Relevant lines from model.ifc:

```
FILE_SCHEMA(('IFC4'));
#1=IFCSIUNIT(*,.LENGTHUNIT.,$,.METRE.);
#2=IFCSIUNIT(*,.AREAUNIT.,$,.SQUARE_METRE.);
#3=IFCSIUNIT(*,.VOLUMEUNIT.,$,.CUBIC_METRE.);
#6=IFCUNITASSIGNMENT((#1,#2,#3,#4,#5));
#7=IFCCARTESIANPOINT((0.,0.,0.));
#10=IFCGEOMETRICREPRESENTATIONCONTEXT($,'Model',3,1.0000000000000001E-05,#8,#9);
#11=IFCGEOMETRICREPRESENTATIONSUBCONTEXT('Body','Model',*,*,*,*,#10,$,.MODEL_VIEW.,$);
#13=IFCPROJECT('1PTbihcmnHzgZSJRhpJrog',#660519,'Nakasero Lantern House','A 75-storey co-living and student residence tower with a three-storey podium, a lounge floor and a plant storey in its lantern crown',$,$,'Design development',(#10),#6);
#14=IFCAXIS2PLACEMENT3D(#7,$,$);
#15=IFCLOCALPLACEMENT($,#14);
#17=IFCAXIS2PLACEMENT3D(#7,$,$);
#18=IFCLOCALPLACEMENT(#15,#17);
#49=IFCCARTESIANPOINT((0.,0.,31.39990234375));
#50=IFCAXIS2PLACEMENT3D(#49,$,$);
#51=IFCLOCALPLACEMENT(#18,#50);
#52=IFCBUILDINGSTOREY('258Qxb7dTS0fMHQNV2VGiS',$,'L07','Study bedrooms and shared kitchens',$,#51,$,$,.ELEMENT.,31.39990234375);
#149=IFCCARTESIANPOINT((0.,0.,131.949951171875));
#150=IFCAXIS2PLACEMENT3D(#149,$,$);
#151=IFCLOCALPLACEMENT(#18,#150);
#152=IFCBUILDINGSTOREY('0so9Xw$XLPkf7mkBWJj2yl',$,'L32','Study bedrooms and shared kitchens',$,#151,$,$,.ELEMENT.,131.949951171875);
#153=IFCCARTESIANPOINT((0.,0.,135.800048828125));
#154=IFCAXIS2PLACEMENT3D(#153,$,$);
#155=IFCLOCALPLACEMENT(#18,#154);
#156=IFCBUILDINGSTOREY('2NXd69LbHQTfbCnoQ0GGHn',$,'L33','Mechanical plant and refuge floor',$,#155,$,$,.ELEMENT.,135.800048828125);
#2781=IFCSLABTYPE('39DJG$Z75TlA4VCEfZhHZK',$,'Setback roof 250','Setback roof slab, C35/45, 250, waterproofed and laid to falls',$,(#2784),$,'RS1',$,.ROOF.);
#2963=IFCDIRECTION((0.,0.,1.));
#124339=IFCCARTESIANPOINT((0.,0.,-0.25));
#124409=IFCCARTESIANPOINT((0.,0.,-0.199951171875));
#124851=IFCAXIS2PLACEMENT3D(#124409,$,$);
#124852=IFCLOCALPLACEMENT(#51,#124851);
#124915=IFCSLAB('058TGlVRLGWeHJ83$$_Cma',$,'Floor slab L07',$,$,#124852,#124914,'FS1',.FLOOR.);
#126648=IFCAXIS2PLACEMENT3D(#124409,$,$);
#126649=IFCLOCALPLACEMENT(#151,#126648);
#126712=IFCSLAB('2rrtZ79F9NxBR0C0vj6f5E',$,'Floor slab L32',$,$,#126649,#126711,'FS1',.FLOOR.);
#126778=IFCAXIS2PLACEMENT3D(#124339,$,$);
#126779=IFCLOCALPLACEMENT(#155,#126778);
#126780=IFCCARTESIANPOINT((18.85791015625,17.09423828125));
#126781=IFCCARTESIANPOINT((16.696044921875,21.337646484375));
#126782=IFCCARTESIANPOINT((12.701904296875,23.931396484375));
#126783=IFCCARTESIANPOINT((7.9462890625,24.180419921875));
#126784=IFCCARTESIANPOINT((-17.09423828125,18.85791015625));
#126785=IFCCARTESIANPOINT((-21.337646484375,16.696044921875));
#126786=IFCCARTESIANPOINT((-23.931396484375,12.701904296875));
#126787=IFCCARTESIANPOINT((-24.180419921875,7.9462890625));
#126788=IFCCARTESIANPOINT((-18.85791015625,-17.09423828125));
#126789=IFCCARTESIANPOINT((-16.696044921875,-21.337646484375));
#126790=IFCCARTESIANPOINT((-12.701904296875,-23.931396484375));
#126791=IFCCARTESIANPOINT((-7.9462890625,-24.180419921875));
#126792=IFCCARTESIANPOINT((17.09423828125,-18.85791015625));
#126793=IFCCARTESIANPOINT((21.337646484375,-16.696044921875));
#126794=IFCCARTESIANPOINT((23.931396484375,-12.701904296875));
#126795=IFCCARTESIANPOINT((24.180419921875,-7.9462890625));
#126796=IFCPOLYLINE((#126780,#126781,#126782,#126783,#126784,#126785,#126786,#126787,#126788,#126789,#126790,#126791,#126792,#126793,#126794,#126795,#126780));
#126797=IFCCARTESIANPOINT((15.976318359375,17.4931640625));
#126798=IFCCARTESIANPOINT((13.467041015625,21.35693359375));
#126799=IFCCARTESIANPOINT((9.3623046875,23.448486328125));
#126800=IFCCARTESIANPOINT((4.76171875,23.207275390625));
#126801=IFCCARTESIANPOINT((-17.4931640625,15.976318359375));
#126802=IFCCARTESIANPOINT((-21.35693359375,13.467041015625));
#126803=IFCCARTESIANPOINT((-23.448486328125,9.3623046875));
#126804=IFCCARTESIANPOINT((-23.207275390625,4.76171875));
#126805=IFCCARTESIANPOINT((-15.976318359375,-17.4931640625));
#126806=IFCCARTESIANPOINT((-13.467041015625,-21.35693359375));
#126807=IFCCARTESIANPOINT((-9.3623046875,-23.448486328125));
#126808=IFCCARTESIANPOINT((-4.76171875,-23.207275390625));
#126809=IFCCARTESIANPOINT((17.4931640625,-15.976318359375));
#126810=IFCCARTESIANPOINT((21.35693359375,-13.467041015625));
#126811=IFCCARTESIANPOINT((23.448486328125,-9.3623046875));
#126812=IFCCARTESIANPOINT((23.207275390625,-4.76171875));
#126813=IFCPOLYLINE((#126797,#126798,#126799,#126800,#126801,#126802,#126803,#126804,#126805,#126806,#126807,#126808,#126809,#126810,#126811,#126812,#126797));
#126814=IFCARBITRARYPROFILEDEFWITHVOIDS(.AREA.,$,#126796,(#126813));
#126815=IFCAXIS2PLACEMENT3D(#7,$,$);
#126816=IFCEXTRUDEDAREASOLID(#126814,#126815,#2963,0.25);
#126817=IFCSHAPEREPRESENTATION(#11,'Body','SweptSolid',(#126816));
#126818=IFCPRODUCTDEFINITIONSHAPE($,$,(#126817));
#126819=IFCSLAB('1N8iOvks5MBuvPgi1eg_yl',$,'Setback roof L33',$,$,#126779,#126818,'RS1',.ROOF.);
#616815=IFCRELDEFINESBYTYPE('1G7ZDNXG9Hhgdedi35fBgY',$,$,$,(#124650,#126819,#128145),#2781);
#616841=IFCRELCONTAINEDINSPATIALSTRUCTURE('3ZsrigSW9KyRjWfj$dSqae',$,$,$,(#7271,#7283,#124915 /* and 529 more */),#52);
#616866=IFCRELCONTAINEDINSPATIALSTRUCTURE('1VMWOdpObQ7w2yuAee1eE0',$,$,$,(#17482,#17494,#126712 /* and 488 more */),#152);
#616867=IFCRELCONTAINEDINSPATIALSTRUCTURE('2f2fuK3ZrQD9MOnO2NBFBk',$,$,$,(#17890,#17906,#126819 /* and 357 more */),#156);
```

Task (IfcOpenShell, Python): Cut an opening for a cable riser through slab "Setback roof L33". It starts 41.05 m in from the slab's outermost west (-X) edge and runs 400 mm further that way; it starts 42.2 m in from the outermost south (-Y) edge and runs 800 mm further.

```python
import numpy as np
import ifcopenshell
import ifcopenshell.api.feature
import ifcopenshell.api.geometry
import ifcopenshell.api.root
import ifcopenshell.geom
import ifcopenshell.util.placement
import ifcopenshell.util.representation
import ifcopenshell.util.shape
import ifcopenshell.util.unit

model = ifcopenshell.open("model.ifc")
unit_scale = ifcopenshell.util.unit.calculate_unit_scale(model)
settings = ifcopenshell.geom.settings()


def volume(element):
    """Net volume in cubic metres, openings subtracted."""
    shape = ifcopenshell.geom.create_shape(settings, element)
    return ifcopenshell.util.shape.get_volume(shape.geometry)


slab = model.by_guid("1N8iOvks5MBuvPgi1eg_yl")
before = volume(slab)

# Extent in the slab's own axes, in metres. The edges named are its -X and -Y sides.
slab_shape = ifcopenshell.geom.create_shape(settings, slab)
vertices = ifcopenshell.util.shape.get_vertices(slab_shape.geometry)
x_min, y_min, bottom = vertices.min(axis=0)
top = vertices[:, 2].max()

opening = ifcopenshell.api.root.create_entity(model, ifc_class="IfcOpeningElement", name="Cable riser opening", predefined_type="OPENING")
context = ifcopenshell.util.representation.get_context(model, "Model", "Body", "MODEL_VIEW")
width, depth = 0.4, 0.8
outline = [(0.0, 0.0), (width, 0.0), (width, depth), (0.0, depth), (0.0, 0.0)]
# Overshoot both faces by 50 mm so the cut is clean.
shape = ifcopenshell.api.geometry.add_slab_representation(
    model, context=context, depth=top - bottom + 0.1, polyline=outline
)
ifcopenshell.api.geometry.assign_representation(model, product=opening, representation=shape)

matrix = ifcopenshell.util.placement.get_local_placement(slab.ObjectPlacement)
matrix[:, 3] = matrix @ np.append(np.array([x_min + 41.05, y_min + 42.2, bottom - 0.05]) / unit_scale, 1.0)
ifcopenshell.api.geometry.edit_object_placement(model, product=opening, matrix=matrix, is_si=False)
ifcopenshell.api.feature.add_feature(model, feature=opening, element=slab)

after = volume(slab)

print(f"slab volume {before:.3f} -> {after:.3f} m3")

model.write("model_rev.ifc")
```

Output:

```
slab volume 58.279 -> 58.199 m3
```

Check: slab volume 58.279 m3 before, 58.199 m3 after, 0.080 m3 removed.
